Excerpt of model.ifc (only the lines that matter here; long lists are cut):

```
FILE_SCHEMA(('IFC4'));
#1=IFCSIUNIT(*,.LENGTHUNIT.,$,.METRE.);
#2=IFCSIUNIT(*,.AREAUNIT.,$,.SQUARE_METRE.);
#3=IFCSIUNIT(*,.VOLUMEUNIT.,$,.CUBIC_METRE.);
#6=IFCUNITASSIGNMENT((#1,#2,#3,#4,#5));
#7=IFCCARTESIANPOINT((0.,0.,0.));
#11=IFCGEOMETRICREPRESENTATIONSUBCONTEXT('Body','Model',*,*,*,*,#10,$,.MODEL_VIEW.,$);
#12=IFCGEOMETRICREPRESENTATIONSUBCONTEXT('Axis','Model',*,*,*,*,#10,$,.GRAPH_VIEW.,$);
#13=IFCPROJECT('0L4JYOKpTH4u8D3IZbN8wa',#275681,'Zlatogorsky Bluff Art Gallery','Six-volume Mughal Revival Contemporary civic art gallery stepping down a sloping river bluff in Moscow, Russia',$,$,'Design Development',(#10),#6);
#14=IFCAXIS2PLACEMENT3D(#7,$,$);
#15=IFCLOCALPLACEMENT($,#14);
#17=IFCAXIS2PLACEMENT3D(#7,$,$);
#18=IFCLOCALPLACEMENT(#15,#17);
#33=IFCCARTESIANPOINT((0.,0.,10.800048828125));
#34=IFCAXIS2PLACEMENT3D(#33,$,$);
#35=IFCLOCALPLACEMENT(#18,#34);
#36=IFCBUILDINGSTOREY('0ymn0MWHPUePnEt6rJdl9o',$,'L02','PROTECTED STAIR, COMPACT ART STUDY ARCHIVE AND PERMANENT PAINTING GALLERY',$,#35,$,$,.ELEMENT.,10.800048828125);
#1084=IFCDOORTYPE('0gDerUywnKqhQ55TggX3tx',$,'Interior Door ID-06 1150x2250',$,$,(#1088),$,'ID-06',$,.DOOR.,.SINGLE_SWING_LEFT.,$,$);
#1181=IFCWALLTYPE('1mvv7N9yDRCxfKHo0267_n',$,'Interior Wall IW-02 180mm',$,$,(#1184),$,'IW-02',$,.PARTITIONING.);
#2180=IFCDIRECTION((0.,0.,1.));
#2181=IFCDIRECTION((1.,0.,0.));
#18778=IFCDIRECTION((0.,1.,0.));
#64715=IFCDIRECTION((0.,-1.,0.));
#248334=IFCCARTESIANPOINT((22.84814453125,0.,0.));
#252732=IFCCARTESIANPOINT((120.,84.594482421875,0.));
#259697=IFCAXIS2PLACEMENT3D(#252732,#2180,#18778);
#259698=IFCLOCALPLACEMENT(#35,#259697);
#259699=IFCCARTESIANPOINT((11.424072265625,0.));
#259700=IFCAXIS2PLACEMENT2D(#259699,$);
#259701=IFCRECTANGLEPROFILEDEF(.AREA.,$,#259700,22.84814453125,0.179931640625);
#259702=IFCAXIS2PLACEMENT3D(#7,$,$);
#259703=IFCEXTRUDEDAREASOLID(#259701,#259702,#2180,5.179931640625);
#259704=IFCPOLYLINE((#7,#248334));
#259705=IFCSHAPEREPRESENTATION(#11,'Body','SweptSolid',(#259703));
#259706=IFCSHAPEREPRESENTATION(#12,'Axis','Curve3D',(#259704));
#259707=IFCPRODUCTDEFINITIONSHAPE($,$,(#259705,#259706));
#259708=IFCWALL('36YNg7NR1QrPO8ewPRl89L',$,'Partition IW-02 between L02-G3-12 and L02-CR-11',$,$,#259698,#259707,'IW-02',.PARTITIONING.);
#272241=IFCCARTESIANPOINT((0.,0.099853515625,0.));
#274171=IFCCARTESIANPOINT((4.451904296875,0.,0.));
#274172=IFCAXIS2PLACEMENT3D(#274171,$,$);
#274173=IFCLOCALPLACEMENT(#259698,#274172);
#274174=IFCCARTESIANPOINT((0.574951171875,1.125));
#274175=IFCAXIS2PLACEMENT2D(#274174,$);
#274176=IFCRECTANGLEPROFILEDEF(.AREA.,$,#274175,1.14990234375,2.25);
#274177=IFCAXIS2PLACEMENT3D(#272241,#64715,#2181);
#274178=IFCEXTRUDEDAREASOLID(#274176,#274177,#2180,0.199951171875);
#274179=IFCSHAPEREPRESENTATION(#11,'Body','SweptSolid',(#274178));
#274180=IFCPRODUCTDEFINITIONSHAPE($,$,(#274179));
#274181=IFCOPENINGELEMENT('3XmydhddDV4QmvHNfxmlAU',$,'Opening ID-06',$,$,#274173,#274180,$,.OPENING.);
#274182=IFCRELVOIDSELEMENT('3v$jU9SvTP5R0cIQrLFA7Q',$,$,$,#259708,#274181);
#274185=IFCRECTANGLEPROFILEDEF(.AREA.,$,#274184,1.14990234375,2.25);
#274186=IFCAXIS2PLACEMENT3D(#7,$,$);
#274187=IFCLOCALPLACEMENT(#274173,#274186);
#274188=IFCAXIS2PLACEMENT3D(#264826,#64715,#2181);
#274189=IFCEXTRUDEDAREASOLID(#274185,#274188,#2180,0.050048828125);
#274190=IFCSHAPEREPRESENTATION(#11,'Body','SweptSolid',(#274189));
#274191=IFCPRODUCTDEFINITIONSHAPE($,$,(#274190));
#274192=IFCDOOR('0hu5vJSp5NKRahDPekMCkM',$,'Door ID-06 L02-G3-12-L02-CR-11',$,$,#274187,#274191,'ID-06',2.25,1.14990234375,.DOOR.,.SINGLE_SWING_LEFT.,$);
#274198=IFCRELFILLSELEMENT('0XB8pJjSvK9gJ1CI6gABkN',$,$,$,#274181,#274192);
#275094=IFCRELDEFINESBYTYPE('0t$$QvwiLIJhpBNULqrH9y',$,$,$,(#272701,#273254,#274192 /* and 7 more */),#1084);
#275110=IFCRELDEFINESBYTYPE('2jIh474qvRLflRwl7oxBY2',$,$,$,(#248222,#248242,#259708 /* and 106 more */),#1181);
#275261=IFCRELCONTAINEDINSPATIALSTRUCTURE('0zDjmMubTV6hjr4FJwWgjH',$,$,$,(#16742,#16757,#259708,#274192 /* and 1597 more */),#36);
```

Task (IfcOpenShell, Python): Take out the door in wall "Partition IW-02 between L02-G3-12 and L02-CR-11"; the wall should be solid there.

```python
import ifcopenshell
import ifcopenshell.api.feature
import ifcopenshell.api.root
import ifcopenshell.geom
import ifcopenshell.util.shape

model = ifcopenshell.open("model.ifc")
settings = ifcopenshell.geom.settings()


def volume(element):
    """Net volume in cubic metres, openings subtracted."""
    shape = ifcopenshell.geom.create_shape(settings, element)
    return ifcopenshell.util.shape.get_volume(shape.geometry)


door = model.by_guid("0hu5vJSp5NKRahDPekMCkM")
opening = door.FillsVoids[0].RelatingOpeningElement
wall = opening.VoidsElements[0].RelatingBuildingElement
before = volume(wall)

ifcopenshell.api.root.remove_product(model, product=door)
ifcopenshell.api.feature.remove_feature(model, feature=opening)

after = volume(wall)

print(f"wall volume {before:.3f} -> {after:.3f} m3")

model.write("model_updated.ifc")
```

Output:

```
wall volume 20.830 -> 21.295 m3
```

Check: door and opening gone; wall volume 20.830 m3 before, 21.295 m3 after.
